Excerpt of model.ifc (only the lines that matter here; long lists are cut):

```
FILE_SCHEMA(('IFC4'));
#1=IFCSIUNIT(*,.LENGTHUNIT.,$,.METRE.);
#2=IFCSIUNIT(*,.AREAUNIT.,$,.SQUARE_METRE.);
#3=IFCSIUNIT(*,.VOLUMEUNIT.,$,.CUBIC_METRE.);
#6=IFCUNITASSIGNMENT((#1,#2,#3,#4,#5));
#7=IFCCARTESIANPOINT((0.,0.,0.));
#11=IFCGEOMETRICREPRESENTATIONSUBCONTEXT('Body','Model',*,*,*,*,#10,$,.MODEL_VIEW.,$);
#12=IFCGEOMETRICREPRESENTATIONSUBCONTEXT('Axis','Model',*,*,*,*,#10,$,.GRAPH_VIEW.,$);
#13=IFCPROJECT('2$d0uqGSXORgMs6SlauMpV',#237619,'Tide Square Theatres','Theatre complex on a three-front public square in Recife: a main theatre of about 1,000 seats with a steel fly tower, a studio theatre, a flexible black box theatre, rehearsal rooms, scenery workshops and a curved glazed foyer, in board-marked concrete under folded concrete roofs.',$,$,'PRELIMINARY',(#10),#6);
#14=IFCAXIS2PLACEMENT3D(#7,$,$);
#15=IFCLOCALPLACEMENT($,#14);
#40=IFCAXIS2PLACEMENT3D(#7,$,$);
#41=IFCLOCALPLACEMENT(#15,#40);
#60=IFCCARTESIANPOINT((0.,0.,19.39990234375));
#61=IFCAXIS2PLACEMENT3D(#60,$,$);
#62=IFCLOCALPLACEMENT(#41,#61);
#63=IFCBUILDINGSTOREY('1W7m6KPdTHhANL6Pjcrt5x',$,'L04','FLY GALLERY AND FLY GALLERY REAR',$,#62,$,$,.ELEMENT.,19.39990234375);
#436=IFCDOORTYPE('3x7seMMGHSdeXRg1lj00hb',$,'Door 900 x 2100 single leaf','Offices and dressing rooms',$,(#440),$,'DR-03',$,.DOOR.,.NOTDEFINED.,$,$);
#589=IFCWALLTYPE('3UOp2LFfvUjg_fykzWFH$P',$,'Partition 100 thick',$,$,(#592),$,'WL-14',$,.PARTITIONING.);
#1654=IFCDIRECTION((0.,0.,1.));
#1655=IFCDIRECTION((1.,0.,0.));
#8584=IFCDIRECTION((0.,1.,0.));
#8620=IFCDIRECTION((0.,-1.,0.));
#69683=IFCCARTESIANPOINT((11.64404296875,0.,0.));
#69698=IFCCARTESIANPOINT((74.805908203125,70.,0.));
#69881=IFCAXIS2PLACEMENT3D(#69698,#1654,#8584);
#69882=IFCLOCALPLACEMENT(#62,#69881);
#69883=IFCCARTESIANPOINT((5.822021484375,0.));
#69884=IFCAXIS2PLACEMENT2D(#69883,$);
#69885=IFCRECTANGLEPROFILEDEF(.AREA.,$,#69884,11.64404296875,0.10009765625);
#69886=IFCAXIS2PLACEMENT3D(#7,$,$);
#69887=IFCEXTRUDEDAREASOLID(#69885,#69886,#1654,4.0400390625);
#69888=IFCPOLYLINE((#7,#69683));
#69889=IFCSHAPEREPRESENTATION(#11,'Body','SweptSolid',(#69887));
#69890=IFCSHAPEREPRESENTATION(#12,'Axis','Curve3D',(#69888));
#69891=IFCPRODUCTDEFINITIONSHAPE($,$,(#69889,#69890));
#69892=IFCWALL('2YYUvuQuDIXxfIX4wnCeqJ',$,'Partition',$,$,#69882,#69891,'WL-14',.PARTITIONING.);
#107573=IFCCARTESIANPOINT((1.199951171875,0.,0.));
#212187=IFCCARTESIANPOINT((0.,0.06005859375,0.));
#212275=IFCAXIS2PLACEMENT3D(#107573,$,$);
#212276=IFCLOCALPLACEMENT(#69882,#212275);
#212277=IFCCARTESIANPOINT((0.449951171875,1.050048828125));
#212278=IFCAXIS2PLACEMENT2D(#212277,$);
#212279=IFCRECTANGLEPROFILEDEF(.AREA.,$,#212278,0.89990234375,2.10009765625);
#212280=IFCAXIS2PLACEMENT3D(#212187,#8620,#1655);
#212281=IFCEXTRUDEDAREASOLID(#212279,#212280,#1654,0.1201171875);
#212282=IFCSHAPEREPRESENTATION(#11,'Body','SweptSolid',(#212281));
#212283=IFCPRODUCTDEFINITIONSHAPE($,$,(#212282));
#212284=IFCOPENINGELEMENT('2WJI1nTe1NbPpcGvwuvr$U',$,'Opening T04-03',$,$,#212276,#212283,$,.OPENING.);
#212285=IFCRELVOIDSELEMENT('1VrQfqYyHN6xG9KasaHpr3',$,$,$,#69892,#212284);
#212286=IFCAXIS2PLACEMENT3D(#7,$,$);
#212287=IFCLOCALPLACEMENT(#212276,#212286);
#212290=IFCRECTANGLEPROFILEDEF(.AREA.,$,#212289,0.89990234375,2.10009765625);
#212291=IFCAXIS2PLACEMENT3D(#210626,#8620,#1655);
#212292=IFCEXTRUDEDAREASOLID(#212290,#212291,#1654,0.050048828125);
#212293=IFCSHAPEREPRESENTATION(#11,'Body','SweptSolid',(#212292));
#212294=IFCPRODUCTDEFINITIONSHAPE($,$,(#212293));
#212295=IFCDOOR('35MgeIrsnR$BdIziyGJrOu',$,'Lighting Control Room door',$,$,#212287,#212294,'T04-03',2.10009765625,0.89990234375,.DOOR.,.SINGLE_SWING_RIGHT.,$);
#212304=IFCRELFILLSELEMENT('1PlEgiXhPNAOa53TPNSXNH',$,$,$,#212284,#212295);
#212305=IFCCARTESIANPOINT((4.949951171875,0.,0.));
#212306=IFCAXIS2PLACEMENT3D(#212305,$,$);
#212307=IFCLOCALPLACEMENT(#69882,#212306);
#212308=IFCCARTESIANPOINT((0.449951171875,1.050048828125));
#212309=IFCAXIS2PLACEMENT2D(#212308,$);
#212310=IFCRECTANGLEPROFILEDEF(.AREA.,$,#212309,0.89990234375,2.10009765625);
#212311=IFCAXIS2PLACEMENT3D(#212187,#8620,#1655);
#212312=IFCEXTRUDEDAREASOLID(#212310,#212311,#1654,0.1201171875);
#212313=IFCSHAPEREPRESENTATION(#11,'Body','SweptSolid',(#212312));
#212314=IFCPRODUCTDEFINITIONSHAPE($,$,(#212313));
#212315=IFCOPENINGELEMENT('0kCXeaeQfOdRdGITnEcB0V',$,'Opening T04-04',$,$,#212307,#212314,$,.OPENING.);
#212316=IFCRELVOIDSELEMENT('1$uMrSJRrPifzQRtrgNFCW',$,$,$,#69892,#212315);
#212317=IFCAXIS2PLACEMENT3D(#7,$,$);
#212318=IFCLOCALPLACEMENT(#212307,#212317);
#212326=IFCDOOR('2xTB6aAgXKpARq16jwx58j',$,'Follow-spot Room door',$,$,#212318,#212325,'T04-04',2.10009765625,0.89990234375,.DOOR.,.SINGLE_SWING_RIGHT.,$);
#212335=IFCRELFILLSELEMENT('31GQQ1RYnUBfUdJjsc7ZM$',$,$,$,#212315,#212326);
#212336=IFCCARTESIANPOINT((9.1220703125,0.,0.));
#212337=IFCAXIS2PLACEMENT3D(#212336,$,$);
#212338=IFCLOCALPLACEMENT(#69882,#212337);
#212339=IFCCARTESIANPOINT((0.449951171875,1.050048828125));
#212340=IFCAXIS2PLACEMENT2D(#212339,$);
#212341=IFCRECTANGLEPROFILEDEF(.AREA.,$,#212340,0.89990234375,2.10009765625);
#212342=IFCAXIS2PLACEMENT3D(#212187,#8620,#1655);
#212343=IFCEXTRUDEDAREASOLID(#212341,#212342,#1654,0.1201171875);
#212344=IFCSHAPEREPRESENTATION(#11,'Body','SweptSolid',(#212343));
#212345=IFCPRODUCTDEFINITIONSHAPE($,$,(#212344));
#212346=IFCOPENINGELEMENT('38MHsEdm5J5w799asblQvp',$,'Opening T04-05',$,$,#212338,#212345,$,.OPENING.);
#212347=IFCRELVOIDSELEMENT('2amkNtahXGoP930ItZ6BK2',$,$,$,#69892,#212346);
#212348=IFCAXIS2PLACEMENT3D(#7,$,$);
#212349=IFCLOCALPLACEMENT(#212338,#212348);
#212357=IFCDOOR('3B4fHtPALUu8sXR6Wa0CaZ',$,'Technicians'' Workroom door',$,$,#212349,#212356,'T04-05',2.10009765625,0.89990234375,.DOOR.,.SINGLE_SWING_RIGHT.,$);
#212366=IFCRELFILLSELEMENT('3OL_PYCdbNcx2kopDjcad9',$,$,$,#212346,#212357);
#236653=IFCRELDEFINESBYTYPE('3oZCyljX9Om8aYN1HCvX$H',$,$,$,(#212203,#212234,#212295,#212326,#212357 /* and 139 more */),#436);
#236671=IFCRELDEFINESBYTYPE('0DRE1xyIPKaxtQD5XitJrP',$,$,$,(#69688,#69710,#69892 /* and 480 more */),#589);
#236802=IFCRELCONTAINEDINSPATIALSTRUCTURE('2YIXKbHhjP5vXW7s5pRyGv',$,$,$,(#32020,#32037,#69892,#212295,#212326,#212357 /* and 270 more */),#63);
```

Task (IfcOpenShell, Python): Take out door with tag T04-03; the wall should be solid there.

```python
import ifcopenshell
import ifcopenshell.api.feature
import ifcopenshell.api.root
import ifcopenshell.geom
import ifcopenshell.util.shape

model = ifcopenshell.open("model.ifc")
settings = ifcopenshell.geom.settings()


def volume(element):
    """Net volume in cubic metres, openings subtracted."""
    shape = ifcopenshell.geom.create_shape(settings, element)
    return ifcopenshell.util.shape.get_volume(shape.geometry)


door = model.by_guid("35MgeIrsnR$BdIziyGJrOu")
opening = door.FillsVoids[0].RelatingOpeningElement
wall = opening.VoidsElements[0].RelatingBuildingElement
before = volume(wall)

ifcopenshell.api.root.remove_product(model, product=door)
ifcopenshell.api.feature.remove_feature(model, feature=opening)

after = volume(wall)

print(f"wall volume {before:.3f} -> {after:.3f} m3")

model.write("model_edited.ifc")
```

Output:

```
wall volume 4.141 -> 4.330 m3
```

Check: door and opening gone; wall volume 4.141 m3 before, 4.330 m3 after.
